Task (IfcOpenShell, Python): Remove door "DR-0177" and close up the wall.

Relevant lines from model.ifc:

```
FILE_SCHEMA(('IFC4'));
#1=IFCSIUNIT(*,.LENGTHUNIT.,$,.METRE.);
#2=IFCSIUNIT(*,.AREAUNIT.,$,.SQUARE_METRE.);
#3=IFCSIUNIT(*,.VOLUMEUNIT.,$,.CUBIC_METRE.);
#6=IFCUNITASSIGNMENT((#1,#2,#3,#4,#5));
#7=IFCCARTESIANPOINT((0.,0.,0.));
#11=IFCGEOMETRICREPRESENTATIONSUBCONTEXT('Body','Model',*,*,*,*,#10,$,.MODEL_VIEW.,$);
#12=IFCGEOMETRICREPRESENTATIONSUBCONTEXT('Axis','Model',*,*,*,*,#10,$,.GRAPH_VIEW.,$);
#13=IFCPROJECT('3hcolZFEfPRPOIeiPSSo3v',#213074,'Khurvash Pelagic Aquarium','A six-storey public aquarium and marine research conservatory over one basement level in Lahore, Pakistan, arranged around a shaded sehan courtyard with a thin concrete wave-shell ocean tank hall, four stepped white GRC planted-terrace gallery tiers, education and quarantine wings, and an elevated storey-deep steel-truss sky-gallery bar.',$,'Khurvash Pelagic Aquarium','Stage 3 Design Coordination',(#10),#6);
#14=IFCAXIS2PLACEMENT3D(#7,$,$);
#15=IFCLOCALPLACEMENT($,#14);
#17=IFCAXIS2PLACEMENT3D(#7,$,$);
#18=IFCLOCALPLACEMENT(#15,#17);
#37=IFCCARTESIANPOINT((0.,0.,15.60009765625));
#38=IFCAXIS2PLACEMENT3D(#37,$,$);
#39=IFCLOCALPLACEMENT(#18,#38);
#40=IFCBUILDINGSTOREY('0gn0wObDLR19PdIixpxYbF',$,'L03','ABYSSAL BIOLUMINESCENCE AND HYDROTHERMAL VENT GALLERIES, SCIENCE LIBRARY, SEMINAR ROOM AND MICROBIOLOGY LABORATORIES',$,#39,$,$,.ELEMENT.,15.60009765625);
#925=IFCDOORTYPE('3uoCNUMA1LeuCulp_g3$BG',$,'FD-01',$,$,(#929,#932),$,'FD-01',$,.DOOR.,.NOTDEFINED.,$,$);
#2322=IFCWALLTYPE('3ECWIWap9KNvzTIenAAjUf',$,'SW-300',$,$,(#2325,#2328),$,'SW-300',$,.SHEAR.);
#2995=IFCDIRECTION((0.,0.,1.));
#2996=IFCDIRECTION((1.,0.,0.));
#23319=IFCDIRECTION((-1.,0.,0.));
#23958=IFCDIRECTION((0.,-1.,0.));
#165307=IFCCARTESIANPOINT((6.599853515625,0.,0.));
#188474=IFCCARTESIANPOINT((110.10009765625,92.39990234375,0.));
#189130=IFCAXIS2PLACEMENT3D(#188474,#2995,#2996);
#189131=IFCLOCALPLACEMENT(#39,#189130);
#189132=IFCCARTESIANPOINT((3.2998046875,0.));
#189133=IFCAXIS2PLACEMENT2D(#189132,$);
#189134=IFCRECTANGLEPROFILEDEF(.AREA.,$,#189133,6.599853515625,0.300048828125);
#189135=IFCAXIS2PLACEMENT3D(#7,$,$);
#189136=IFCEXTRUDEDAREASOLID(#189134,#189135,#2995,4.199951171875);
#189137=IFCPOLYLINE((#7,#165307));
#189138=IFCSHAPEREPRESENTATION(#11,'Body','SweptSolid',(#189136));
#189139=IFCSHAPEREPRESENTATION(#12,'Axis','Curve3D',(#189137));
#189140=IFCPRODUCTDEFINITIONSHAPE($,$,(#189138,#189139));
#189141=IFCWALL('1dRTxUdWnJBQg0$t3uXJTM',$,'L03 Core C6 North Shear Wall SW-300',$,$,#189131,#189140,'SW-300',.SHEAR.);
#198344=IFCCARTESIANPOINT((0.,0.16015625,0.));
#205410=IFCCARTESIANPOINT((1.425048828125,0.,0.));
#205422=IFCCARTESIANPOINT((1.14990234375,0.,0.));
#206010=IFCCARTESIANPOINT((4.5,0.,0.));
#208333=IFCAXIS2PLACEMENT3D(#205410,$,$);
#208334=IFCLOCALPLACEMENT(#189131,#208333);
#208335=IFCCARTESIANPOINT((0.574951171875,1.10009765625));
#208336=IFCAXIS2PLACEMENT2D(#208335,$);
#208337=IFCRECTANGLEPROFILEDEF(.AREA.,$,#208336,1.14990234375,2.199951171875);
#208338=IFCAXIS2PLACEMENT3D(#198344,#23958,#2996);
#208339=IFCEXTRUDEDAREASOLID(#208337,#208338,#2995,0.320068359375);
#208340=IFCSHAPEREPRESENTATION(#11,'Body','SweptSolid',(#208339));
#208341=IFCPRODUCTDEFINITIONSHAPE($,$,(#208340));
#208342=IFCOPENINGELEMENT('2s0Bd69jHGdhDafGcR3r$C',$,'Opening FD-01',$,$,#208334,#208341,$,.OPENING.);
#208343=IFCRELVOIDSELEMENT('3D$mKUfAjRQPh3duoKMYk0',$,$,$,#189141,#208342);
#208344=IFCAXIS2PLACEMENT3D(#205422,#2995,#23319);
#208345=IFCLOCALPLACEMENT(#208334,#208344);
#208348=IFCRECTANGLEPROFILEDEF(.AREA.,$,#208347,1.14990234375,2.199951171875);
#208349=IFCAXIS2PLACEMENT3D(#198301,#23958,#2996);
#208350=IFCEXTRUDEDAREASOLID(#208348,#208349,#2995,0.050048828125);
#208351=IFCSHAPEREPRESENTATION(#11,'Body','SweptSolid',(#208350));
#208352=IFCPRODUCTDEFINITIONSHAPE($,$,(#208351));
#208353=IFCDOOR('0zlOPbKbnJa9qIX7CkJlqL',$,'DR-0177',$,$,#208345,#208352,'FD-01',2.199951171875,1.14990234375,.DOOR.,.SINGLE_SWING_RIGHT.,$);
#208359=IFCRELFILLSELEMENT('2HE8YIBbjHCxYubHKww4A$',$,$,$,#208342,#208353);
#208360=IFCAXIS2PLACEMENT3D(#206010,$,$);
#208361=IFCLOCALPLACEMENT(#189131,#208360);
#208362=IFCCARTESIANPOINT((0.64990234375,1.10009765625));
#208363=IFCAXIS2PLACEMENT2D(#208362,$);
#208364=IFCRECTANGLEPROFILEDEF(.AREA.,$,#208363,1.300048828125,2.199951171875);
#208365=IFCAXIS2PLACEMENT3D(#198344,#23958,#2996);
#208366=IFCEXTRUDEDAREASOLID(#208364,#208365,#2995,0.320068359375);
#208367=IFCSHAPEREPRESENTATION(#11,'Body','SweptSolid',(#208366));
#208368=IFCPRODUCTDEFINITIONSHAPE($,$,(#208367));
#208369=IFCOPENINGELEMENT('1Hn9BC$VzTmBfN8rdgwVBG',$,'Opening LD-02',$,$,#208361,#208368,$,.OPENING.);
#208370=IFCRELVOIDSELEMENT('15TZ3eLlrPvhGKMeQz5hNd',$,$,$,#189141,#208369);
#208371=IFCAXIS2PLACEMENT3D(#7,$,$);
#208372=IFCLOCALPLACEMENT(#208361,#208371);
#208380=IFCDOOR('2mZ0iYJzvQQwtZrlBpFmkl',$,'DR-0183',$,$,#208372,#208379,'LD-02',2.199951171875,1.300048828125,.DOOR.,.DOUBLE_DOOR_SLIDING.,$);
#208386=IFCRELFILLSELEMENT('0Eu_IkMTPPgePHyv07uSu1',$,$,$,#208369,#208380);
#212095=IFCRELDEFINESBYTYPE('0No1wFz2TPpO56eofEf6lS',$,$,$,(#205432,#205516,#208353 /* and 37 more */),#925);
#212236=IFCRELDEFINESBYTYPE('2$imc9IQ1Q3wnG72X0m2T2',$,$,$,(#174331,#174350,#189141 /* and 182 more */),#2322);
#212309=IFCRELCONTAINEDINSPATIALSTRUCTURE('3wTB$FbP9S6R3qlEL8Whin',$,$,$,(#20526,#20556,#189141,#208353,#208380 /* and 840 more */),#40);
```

```python
import ifcopenshell
import ifcopenshell.api.feature
import ifcopenshell.api.root
import ifcopenshell.geom
import ifcopenshell.util.shape

model = ifcopenshell.open("model.ifc")
settings = ifcopenshell.geom.settings()


def volume(element):
    """Net volume in cubic metres, openings subtracted."""
    shape = ifcopenshell.geom.create_shape(settings, element)
    return ifcopenshell.util.shape.get_volume(shape.geometry)


door = model.by_guid("0zlOPbKbnJa9qIX7CkJlqL")
opening = door.FillsVoids[0].RelatingOpeningElement
wall = opening.VoidsElements[0].RelatingBuildingElement
before = volume(wall)

ifcopenshell.api.root.remove_product(model, product=door)
ifcopenshell.api.feature.remove_feature(model, feature=opening)

after = volume(wall)

print(f"wall volume {before:.3f} -> {after:.3f} m3")

model.write("model_v2.ifc")
```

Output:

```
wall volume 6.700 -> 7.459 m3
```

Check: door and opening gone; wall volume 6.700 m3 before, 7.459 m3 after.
